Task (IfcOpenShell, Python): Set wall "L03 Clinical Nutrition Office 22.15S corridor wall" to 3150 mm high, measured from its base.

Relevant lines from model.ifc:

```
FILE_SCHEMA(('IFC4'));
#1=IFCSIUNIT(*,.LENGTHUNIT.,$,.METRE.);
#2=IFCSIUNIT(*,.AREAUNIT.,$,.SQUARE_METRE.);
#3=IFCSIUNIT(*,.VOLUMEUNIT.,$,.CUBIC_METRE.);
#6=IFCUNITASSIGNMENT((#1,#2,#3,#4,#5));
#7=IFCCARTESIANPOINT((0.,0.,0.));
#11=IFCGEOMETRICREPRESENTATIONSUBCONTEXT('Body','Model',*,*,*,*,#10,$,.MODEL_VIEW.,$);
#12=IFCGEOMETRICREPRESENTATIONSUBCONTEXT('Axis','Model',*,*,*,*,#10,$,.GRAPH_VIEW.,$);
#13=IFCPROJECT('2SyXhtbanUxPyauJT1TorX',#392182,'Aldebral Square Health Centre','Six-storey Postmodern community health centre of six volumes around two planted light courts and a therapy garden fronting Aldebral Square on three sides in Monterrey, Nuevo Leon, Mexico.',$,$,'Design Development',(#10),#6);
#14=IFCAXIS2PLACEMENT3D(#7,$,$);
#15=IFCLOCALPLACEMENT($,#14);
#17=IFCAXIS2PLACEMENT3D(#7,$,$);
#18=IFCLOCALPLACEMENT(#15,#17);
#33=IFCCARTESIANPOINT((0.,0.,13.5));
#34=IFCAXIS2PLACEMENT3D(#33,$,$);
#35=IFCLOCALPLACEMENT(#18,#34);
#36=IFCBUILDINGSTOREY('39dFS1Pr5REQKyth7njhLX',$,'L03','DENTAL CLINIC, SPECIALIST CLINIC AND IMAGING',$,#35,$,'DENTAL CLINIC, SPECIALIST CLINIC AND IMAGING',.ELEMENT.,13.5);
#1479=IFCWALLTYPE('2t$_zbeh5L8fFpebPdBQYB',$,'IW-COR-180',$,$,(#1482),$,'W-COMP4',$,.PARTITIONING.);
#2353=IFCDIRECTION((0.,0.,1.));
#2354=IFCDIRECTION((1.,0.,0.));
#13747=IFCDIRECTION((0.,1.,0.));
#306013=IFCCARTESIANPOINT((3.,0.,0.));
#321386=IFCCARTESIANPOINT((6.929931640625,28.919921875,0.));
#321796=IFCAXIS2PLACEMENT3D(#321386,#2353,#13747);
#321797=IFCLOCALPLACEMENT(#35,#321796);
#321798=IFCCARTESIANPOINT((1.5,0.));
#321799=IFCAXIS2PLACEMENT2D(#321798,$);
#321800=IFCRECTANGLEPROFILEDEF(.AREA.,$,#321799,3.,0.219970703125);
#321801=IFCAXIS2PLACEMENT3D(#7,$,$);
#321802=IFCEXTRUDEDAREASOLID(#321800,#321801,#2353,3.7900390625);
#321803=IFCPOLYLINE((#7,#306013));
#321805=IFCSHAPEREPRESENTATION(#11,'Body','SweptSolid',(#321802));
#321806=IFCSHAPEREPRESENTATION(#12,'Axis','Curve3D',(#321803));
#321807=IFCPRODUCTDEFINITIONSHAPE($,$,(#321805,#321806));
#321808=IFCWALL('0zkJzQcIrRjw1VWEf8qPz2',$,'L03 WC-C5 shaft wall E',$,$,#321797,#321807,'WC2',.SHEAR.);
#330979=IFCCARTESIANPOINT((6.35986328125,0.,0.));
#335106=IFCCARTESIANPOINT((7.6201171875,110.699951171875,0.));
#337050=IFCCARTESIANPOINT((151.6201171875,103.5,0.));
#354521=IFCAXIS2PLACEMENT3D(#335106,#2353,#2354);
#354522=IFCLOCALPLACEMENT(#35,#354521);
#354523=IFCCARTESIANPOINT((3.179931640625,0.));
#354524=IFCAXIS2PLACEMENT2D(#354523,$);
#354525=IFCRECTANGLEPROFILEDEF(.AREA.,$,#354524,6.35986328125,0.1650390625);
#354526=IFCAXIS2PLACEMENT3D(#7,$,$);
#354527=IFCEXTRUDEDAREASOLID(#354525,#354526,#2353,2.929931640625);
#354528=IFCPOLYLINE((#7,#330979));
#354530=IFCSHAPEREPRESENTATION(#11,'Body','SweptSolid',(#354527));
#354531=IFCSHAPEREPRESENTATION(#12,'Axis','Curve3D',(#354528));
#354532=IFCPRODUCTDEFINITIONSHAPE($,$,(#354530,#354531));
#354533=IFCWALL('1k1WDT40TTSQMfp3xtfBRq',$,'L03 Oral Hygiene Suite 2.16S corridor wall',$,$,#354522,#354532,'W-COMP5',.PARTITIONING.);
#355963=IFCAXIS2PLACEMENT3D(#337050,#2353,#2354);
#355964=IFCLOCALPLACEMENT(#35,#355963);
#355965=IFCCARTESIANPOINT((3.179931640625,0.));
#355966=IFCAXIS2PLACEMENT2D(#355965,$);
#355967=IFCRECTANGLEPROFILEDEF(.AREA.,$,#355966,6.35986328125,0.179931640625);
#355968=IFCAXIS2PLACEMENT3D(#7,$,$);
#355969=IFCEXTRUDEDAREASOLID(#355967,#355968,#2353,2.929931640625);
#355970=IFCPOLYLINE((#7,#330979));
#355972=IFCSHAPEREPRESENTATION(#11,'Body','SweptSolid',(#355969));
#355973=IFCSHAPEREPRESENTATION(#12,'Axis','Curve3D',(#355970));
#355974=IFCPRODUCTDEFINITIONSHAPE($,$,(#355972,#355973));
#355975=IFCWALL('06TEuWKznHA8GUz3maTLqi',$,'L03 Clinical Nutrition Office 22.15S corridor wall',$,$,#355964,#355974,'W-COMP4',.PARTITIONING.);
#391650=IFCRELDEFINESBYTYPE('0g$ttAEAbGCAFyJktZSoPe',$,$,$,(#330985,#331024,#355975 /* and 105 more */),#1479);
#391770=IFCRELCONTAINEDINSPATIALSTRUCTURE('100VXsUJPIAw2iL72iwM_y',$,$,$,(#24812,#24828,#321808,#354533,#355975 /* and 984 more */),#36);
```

```python
import ifcopenshell
import ifcopenshell.geom
import ifcopenshell.util.representation
import ifcopenshell.util.shape

model = ifcopenshell.open("model.ifc")
settings = ifcopenshell.geom.settings()


def volume(element):
    """Net volume in cubic metres, openings subtracted."""
    shape = ifcopenshell.geom.create_shape(settings, element)
    return ifcopenshell.util.shape.get_volume(shape.geometry)


wall = model.by_guid("06TEuWKznHA8GUz3maTLqi")
before = volume(wall)

body = ifcopenshell.util.representation.get_representation(wall, "Model", "Body")
solid = body.Items[0]
old_height = solid.Depth
solid.Depth = 3.15
after = volume(wall)

print(f"height {old_height:g} -> {solid.Depth:g}, volume {before:.3f} -> {after:.3f} m3")

model.write("model_edited.ifc")
```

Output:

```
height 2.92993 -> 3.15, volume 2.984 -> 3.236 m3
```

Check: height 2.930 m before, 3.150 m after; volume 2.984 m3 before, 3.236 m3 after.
